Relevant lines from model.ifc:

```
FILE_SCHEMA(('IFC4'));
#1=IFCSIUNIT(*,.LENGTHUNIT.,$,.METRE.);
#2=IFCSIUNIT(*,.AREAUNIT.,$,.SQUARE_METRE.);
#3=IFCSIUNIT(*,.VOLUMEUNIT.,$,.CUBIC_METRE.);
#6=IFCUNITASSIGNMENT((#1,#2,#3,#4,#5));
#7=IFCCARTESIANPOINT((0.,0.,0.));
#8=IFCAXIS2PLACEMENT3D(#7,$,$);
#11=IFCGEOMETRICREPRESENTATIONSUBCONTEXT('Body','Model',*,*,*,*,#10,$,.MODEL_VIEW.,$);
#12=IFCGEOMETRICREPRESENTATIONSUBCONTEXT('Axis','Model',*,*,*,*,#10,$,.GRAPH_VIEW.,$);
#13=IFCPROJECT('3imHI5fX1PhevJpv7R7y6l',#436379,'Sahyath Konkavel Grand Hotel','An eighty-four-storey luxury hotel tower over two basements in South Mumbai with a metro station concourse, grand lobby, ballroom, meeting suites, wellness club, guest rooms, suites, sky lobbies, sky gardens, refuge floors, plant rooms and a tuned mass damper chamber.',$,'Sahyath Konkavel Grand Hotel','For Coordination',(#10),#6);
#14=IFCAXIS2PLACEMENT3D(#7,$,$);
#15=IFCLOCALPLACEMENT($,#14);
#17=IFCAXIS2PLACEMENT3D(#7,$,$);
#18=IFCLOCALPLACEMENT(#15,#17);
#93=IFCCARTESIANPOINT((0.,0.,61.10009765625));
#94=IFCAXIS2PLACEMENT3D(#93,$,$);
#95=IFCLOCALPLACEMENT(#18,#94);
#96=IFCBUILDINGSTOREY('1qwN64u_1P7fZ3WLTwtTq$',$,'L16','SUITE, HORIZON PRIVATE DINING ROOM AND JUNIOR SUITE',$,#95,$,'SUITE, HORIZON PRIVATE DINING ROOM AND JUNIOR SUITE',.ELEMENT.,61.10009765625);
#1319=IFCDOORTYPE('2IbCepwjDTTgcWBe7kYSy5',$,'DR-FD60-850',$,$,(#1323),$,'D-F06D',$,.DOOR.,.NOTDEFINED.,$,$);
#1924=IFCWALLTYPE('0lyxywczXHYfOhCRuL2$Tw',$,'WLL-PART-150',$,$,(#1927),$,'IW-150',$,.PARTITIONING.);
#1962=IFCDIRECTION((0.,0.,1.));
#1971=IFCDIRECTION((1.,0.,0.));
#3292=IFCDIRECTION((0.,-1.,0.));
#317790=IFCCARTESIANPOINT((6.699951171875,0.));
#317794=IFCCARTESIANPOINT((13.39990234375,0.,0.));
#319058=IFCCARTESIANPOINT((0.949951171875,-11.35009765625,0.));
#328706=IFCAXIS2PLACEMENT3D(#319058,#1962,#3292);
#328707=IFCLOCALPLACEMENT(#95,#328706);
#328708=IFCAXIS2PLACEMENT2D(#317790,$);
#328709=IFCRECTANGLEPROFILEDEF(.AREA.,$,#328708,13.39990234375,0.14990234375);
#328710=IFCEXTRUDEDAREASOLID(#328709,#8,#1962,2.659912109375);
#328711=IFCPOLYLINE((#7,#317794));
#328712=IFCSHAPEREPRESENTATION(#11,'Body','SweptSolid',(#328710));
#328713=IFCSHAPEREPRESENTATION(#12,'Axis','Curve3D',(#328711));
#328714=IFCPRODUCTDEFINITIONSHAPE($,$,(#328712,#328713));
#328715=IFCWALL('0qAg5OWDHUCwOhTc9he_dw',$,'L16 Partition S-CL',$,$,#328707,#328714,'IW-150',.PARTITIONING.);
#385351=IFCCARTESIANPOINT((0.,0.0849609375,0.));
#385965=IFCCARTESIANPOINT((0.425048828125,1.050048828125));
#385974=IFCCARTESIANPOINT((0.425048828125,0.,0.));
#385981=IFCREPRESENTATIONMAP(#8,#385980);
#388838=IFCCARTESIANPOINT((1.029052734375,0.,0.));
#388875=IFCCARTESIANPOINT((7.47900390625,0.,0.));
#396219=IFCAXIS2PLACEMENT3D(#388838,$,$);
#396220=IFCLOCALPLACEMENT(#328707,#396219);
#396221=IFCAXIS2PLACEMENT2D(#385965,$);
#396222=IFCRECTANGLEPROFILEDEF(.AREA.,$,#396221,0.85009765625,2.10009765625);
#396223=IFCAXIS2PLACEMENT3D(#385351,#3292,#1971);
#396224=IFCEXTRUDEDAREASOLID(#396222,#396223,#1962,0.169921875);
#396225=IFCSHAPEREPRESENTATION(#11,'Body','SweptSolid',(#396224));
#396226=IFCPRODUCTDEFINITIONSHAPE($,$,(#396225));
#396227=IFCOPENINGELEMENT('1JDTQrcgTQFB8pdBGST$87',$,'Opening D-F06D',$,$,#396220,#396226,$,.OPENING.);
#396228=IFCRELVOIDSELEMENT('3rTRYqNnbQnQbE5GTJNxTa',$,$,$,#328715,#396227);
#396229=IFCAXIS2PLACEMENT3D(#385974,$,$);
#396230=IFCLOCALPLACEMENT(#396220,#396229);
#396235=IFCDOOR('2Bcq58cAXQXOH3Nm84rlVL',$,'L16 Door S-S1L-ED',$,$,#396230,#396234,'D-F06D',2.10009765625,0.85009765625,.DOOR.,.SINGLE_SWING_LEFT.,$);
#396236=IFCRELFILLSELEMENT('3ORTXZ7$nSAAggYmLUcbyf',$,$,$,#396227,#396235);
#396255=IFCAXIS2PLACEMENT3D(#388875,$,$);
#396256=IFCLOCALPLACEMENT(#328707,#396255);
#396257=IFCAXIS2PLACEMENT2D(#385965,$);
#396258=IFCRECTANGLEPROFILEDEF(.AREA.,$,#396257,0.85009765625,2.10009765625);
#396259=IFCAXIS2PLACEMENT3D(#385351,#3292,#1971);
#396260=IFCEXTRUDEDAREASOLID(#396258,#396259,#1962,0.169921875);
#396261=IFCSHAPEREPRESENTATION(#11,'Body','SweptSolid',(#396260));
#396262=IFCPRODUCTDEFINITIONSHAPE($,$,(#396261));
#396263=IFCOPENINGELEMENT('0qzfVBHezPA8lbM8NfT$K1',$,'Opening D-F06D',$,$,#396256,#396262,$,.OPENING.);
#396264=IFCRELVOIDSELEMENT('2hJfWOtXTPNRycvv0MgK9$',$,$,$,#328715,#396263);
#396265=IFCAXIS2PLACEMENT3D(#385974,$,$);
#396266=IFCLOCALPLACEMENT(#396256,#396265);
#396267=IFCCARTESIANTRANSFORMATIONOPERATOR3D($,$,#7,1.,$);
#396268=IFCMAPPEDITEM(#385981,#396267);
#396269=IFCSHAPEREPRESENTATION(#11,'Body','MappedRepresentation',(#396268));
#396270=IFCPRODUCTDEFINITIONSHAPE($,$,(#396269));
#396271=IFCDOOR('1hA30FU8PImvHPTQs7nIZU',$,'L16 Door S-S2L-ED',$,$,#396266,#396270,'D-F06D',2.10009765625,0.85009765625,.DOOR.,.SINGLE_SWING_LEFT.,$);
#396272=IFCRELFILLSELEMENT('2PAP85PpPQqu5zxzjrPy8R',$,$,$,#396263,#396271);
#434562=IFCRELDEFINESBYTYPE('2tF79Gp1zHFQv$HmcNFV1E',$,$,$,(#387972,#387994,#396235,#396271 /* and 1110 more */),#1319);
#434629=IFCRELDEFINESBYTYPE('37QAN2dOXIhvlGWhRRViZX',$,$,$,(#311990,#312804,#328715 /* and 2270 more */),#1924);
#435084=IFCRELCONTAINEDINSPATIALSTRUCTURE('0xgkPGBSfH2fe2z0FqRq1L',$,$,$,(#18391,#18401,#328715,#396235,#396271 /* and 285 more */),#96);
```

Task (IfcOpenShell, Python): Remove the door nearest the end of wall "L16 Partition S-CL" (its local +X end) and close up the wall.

```python
import ifcopenshell
import ifcopenshell.api.feature
import ifcopenshell.api.root
import ifcopenshell.geom
import ifcopenshell.util.shape

model = ifcopenshell.open("model.ifc")
settings = ifcopenshell.geom.settings()


def volume(element):
    """Net volume in cubic metres, openings subtracted."""
    shape = ifcopenshell.geom.create_shape(settings, element)
    return ifcopenshell.util.shape.get_volume(shape.geometry)


door = model.by_id(396271)
opening = door.FillsVoids[0].RelatingOpeningElement
wall = opening.VoidsElements[0].RelatingBuildingElement
before = volume(wall)

ifcopenshell.api.root.remove_product(model, product=door)
ifcopenshell.api.feature.remove_feature(model, feature=opening)

after = volume(wall)

print(f"wall volume {before:.3f} -> {after:.3f} m3")

model.write("model_edited.ifc")
```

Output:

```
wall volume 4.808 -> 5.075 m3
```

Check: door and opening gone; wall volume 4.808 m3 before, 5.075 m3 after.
